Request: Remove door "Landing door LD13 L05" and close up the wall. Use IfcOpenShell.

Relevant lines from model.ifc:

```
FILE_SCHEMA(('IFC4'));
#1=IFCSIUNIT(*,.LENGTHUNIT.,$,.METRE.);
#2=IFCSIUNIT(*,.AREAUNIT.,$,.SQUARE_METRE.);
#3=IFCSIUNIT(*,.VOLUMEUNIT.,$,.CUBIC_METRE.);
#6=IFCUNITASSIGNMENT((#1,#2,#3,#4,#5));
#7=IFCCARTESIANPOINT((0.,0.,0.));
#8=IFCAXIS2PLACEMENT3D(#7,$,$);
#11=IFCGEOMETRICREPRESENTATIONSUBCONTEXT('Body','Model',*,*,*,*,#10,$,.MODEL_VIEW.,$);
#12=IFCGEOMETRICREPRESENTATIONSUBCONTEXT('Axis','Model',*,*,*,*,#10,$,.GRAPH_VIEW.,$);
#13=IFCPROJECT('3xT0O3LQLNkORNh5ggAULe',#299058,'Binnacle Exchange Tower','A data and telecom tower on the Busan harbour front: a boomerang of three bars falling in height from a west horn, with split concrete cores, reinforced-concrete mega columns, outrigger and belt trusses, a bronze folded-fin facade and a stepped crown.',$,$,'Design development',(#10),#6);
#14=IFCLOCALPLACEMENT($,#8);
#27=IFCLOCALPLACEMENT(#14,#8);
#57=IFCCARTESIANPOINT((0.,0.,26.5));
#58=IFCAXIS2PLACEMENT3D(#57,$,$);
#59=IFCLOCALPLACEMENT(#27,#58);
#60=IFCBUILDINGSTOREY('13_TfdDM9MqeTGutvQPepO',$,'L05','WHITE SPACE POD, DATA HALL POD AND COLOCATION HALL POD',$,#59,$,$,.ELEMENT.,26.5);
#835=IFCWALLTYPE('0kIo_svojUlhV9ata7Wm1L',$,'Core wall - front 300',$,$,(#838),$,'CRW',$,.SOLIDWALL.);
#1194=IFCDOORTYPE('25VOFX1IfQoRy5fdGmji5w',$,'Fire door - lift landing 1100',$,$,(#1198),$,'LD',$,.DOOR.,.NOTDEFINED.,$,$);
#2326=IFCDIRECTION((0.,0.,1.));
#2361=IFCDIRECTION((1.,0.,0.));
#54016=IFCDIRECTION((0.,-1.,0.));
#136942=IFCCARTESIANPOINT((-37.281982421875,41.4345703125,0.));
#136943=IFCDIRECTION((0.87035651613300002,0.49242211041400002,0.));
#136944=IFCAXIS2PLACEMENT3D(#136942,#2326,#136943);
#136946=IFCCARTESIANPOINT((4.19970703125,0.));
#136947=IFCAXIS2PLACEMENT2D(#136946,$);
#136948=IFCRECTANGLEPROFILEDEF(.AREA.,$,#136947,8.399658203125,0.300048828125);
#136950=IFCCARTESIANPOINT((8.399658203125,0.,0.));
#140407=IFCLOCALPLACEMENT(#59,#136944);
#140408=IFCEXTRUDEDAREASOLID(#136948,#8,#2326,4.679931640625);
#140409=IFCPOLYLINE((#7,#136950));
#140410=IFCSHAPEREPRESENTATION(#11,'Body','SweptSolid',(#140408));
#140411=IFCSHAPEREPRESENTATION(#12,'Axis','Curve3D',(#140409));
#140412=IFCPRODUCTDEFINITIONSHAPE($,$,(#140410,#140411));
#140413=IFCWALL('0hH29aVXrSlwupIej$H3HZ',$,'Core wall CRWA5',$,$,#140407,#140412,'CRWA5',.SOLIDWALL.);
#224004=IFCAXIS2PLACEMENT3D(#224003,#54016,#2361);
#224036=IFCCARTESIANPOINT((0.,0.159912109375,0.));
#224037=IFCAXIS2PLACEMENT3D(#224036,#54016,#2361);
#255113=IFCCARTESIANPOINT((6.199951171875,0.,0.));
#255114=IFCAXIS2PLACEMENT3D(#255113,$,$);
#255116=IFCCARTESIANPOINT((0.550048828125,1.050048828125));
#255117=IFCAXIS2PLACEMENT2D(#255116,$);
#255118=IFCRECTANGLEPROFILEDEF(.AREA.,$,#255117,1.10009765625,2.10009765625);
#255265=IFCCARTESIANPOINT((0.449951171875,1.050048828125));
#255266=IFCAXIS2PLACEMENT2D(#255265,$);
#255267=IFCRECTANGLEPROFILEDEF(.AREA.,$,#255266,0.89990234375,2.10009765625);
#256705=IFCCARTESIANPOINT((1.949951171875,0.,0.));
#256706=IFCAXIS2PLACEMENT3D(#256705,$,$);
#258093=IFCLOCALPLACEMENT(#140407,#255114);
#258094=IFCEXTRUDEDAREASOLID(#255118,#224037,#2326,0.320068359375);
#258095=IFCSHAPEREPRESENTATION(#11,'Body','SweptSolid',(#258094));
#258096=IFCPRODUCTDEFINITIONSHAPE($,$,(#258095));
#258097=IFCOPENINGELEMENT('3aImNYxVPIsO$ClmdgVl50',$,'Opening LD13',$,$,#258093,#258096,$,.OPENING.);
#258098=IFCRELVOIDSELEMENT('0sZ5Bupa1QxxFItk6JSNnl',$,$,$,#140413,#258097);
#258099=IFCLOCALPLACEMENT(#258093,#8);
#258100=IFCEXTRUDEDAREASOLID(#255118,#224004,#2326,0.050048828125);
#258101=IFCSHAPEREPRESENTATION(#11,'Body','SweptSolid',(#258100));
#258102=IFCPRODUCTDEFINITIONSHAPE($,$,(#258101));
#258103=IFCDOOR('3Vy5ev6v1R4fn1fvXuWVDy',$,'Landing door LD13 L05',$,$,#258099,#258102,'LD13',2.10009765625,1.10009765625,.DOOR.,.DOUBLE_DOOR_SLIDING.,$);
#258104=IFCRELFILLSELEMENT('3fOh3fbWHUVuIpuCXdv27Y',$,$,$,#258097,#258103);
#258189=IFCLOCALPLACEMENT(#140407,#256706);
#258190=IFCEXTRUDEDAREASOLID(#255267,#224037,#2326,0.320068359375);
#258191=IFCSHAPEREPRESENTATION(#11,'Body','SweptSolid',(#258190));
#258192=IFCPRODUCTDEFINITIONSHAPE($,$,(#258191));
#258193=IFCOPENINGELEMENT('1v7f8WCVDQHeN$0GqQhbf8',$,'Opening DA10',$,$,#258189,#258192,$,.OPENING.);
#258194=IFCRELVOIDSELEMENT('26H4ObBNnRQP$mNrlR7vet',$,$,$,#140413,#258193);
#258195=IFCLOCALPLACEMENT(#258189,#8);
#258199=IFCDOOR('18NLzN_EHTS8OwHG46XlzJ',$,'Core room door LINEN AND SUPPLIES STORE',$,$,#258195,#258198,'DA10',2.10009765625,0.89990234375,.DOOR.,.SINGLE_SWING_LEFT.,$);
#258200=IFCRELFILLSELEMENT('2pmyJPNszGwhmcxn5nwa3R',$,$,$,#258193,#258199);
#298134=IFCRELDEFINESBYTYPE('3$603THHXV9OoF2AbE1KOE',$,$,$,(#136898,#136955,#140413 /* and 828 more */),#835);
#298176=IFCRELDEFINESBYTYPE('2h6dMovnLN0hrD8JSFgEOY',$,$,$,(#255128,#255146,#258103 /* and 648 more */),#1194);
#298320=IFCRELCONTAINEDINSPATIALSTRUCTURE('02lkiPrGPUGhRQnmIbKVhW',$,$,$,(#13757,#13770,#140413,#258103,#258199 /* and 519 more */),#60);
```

```python
import ifcopenshell
import ifcopenshell.api.feature
import ifcopenshell.api.root
import ifcopenshell.geom
import ifcopenshell.util.shape

model = ifcopenshell.open("model.ifc")
settings = ifcopenshell.geom.settings()


def volume(element):
    """Net volume in cubic metres, openings subtracted."""
    shape = ifcopenshell.geom.create_shape(settings, element)
    return ifcopenshell.util.shape.get_volume(shape.geometry)


door = model.by_id(258103)
opening = door.FillsVoids[0].RelatingOpeningElement
wall = opening.VoidsElements[0].RelatingBuildingElement
before = volume(wall)

ifcopenshell.api.root.remove_product(model, product=door)
ifcopenshell.api.feature.remove_feature(model, feature=opening)

after = volume(wall)

print(f"wall volume {before:.3f} -> {after:.3f} m3")

model.write("model_rev.ifc")
```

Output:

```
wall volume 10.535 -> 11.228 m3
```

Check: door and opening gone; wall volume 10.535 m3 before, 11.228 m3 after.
